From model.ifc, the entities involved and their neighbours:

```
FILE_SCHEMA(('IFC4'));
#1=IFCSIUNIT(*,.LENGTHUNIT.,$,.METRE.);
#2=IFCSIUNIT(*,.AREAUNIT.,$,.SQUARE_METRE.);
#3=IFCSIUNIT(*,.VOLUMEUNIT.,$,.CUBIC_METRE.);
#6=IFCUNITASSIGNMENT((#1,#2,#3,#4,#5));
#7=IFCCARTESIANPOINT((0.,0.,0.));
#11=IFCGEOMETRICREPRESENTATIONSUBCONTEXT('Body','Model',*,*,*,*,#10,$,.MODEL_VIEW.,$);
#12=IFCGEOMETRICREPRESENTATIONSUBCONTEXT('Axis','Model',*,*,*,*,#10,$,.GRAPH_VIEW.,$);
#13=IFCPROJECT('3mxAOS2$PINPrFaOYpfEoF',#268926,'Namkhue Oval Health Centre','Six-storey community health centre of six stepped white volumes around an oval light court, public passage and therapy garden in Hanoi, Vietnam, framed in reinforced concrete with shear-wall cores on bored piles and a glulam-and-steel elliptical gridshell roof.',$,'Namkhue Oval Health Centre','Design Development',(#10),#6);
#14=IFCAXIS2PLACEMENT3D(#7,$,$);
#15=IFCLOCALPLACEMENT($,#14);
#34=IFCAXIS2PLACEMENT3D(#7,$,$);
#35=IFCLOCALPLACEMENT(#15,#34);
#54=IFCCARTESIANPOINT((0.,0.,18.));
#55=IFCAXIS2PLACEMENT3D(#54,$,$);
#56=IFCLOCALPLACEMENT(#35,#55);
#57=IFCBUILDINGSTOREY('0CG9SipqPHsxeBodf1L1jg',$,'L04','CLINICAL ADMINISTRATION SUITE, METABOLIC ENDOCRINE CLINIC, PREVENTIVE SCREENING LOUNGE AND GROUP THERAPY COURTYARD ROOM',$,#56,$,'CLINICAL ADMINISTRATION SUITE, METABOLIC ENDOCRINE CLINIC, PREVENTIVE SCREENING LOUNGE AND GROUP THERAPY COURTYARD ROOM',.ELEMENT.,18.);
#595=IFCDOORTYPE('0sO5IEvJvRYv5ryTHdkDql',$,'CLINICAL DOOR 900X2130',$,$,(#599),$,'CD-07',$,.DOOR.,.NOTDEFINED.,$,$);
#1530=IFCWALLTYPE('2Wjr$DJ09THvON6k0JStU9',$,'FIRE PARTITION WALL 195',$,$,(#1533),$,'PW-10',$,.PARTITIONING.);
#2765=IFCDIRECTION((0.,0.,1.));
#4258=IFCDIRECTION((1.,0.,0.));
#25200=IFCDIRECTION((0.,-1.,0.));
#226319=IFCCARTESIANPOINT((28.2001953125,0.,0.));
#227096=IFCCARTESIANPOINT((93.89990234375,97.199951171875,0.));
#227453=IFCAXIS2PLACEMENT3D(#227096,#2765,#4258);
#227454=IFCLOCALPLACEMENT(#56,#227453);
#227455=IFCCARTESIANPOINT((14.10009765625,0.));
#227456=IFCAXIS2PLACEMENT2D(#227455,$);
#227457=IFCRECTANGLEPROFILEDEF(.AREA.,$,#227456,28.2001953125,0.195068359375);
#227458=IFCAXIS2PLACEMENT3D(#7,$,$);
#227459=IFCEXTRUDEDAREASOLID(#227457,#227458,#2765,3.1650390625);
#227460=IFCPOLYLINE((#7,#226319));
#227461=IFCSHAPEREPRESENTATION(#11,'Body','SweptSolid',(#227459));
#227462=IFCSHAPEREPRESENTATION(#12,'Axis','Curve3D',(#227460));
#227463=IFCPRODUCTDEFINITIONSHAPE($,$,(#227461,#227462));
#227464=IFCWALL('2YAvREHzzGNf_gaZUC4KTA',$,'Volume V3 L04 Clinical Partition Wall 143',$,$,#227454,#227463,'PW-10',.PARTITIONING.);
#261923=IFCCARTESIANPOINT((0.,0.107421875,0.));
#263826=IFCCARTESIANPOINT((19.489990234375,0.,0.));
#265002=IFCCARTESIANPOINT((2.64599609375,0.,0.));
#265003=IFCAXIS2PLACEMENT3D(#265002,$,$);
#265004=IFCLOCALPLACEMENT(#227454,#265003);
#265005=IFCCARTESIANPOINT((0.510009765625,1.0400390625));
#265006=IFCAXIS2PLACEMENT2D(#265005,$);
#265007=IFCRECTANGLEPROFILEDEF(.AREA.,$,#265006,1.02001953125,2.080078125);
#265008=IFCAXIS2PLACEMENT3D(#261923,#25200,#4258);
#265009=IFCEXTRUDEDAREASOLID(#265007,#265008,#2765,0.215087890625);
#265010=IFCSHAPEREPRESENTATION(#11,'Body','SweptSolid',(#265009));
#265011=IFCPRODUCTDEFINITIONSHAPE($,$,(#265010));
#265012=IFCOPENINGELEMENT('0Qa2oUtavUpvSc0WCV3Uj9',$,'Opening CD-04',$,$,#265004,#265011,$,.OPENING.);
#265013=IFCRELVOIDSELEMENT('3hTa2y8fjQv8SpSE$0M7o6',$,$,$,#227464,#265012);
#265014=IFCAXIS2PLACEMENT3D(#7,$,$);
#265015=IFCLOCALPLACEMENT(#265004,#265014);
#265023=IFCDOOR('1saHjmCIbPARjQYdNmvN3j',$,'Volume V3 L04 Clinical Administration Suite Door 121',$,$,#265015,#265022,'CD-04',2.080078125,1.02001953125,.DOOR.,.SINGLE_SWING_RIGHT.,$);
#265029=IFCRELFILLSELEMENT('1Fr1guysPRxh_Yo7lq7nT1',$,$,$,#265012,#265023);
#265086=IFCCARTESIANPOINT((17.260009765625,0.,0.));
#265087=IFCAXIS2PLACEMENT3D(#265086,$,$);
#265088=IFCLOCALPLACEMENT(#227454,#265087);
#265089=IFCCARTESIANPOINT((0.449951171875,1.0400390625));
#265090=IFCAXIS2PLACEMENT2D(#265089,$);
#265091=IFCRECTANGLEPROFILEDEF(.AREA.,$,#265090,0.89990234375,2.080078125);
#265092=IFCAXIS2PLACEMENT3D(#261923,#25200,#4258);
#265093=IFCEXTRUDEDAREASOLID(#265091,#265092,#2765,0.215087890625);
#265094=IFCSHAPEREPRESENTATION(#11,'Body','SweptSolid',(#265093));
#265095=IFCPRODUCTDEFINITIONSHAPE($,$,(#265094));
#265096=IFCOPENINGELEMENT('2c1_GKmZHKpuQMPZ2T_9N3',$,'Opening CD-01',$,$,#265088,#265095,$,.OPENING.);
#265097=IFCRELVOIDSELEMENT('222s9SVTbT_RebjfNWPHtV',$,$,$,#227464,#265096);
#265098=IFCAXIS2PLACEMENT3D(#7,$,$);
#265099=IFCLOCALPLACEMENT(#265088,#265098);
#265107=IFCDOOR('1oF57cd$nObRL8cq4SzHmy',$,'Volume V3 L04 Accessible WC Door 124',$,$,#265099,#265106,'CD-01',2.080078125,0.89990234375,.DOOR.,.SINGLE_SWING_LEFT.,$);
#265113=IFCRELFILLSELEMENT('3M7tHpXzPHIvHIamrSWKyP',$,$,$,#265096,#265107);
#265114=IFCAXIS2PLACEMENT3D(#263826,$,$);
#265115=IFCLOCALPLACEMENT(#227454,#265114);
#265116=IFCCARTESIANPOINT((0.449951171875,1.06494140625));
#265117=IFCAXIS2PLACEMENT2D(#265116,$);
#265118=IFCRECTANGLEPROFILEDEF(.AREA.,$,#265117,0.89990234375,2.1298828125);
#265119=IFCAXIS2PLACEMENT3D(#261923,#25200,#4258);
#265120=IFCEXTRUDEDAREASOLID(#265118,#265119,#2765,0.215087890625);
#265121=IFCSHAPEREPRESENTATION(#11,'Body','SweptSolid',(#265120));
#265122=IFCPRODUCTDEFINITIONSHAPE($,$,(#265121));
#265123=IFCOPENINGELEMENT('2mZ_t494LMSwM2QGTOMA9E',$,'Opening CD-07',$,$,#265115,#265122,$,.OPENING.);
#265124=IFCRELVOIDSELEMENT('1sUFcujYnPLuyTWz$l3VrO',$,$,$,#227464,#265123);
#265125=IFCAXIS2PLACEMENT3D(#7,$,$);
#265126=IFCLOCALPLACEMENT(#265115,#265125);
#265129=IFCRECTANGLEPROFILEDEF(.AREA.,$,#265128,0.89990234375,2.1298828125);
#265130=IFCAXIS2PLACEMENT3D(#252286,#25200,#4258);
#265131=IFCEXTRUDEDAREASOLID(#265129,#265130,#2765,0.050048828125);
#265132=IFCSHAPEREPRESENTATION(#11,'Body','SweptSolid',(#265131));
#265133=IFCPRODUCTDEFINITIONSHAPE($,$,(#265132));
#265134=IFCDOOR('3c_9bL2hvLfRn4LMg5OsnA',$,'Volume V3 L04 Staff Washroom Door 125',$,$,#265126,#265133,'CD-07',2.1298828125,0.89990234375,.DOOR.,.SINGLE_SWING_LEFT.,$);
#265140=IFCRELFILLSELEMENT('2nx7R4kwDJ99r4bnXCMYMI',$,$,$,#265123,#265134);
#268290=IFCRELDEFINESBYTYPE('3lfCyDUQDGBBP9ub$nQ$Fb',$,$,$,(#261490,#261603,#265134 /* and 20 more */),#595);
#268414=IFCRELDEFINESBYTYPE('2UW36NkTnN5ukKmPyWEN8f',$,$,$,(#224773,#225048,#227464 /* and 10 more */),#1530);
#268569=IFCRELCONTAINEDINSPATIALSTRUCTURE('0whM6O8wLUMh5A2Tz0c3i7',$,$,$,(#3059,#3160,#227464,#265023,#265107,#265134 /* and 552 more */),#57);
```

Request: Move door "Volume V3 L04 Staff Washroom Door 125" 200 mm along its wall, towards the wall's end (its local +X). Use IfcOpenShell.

```python
import ifcopenshell
import ifcopenshell.api.geometry
import ifcopenshell.util.placement

model = ifcopenshell.open("model.ifc")

door = model.by_guid("3c_9bL2hvLfRn4LMg5OsnA")
opening = door.FillsVoids[0].RelatingOpeningElement
wall = opening.VoidsElements[0].RelatingBuildingElement

wall_matrix = ifcopenshell.util.placement.get_local_placement(wall.ObjectPlacement)
shift = wall_matrix[:3, 0] * 0.2
before = ifcopenshell.util.placement.get_local_placement(door.ObjectPlacement)[:3, 3].copy()

# The door is placed relative to its opening, so it follows when the opening moves.
matrix = ifcopenshell.util.placement.get_local_placement(opening.ObjectPlacement)
matrix[:3, 3] += shift
ifcopenshell.api.geometry.edit_object_placement(
    model, product=opening, matrix=matrix, is_si=False, should_transform_children=True
)

after = ifcopenshell.util.placement.get_local_placement(door.ObjectPlacement)[:3, 3]
print("door moved by", (after - before).round(3) + 0.0)

model.write("model_updated.ifc")
```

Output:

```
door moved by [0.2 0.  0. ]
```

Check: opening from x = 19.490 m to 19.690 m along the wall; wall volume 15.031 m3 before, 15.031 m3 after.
